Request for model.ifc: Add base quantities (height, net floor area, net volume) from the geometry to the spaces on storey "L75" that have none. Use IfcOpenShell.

First a look at what the model holds.

```python
import ifcopenshell
import ifcopenshell.util.element
import ifcopenshell.util.unit

model = ifcopenshell.open("model.ifc")
print(model.schema)
for unit_type in ("LENGTHUNIT", "AREAUNIT", "VOLUMEUNIT"):
    print(unit_type, ifcopenshell.util.unit.calculate_unit_scale(model, unit_type))
storey = next(s for s in model.by_type("IfcBuildingStorey") if s.Name == "L75")
spaces = [e for e in ifcopenshell.util.element.get_decomposition(storey) if e.is_a("IfcSpace")]
for e in sorted(spaces, key=lambda e: e.id()):
    print(e.id(), e.is_a(), e.Name, list(ifcopenshell.util.element.get_psets(e, qtos_only=True)), sep=" | ")
```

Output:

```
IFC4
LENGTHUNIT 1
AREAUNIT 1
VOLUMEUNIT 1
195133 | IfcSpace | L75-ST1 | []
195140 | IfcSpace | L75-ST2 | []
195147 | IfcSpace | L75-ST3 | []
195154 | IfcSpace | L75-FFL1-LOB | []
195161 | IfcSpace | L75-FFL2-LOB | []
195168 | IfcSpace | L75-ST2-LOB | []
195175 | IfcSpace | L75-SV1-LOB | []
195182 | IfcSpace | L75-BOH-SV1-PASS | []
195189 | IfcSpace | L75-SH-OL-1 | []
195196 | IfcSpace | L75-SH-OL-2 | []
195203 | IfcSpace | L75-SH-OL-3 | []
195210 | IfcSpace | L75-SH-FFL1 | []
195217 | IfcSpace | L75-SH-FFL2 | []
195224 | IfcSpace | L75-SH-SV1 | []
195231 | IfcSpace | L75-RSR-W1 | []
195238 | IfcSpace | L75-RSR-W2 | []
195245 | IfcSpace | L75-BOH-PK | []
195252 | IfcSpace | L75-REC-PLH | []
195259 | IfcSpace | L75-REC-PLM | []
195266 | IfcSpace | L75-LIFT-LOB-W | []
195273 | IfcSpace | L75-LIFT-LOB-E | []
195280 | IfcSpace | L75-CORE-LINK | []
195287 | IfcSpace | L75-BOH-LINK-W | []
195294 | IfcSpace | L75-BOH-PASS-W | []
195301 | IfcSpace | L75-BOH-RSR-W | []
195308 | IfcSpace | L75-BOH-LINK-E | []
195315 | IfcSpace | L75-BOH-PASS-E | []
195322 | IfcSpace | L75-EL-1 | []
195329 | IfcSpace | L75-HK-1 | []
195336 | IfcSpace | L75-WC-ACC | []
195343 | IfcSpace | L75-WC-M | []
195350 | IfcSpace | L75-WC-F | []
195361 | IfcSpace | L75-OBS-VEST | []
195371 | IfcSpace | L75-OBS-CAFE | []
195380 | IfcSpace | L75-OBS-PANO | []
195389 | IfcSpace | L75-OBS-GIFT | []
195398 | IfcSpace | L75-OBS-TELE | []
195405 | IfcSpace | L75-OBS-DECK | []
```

```python
import ifcopenshell
import ifcopenshell.api.pset
import ifcopenshell.geom
import ifcopenshell.util.element
import ifcopenshell.util.shape
import ifcopenshell.util.unit

model = ifcopenshell.open("model.ifc")
unit_scale = ifcopenshell.util.unit.calculate_unit_scale(model)
area_scale = ifcopenshell.util.unit.calculate_unit_scale(model, "AREAUNIT")
volume_scale = ifcopenshell.util.unit.calculate_unit_scale(model, "VOLUMEUNIT")
settings = ifcopenshell.geom.settings()

storey = next(s for s in model.by_type("IfcBuildingStorey") if s.Name == "L75")
spaces = [e for e in ifcopenshell.util.element.get_decomposition(storey) if e.is_a("IfcSpace")]

for e in sorted(spaces, key=lambda e: e.id()):
    if ifcopenshell.util.element.get_psets(e, qtos_only=True, should_inherit=False):
        continue
    # Geometry comes back in metres, in the element's own axes.
    shape = ifcopenshell.geom.create_shape(settings, e)
    values = {
        "Height": ifcopenshell.util.shape.get_z(shape.geometry) / unit_scale,
        "NetFloorArea": ifcopenshell.util.shape.get_footprint_area(shape.geometry) / area_scale,
        "NetVolume": ifcopenshell.util.shape.get_volume(shape.geometry) / volume_scale,
    }
    qto = ifcopenshell.api.pset.add_qto(model, product=e, name="Qto_SpaceBaseQuantities")
    ifcopenshell.api.pset.edit_qto(model, qto=qto, properties=values)
    print(e.id(), {k: round(v, 3) for k, v in values.items()})

model.write("model_v2.ifc")
```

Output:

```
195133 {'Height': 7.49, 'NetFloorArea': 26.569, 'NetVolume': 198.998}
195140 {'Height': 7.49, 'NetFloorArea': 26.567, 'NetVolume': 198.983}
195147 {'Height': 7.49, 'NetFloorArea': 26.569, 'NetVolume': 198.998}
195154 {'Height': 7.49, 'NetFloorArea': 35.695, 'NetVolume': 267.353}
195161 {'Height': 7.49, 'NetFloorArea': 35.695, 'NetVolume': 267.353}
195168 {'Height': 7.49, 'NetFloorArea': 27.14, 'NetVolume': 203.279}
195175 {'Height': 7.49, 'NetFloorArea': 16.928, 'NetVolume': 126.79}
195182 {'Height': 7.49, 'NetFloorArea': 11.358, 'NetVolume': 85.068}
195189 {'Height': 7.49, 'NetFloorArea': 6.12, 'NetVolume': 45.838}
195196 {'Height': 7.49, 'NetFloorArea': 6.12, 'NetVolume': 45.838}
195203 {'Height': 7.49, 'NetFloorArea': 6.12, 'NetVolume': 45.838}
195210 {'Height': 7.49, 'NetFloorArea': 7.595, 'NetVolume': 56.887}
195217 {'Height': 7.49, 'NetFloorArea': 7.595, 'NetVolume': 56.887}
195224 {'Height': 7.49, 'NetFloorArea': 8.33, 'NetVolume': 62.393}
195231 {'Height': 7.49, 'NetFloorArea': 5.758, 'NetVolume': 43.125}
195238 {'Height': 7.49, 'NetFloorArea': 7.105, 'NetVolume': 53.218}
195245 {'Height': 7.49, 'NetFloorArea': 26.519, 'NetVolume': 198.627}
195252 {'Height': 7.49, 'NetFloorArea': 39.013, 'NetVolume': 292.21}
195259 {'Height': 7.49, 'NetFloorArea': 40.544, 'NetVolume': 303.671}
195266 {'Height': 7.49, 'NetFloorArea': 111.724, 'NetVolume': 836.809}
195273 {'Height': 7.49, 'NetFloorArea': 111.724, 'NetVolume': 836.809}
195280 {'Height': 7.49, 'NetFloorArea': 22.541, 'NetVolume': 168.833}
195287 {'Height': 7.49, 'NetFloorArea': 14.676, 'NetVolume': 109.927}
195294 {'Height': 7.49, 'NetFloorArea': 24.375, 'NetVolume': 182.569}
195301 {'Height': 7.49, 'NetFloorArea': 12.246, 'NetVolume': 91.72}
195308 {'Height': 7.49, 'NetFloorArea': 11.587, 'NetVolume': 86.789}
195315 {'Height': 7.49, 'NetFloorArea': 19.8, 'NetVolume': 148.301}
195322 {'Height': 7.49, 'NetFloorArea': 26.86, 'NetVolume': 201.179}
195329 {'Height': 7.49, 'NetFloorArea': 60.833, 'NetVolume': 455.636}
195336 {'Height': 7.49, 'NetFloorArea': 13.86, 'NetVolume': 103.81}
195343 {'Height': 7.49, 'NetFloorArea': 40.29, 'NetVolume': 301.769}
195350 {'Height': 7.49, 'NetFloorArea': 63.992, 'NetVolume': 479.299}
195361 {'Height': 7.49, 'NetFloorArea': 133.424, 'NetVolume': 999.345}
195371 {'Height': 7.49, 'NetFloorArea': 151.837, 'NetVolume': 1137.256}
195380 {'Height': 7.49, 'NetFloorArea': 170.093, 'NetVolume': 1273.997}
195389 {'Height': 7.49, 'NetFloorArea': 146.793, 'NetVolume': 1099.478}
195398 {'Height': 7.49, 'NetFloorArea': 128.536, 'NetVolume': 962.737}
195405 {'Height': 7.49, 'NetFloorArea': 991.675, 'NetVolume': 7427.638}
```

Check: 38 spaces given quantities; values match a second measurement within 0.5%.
